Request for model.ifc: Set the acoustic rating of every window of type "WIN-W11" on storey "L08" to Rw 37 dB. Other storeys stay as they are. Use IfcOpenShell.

First a look at what the model holds.

```python
import ifcopenshell
import ifcopenshell.util.element

model = ifcopenshell.open("model.ifc")
print(model.schema)
storey = next(s for s in model.by_type("IfcBuildingStorey") if s.Name == "L08")
windows = [e for e in ifcopenshell.util.element.get_decomposition(storey) if e.is_a("IfcWindow")]
seen = {}
for e in windows:
    element_type = ifcopenshell.util.element.get_type(e)
    key = (element_type.Name if element_type != e and element_type else None, ifcopenshell.util.element.get_pset(e, "Pset_WindowCommon", "AcousticRating"))
    seen[key] = seen.get(key, 0) + 1
for (name, value), count in sorted(seen.items(), key=str):
    print(count, "x", name, "|", value)
```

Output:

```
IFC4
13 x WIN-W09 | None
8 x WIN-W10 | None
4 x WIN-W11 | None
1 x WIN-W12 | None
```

```python
import ifcopenshell
import ifcopenshell.api.pset
import ifcopenshell.util.element

model = ifcopenshell.open("model.ifc")

storey = next(s for s in model.by_type("IfcBuildingStorey") if s.Name == "L08")
windows = [e for e in ifcopenshell.util.element.get_decomposition(storey) if e.is_a("IfcWindow")]

count = 0
for e in windows:
    element_type = ifcopenshell.util.element.get_type(e)
    if element_type in (None, e) or element_type.Name != "WIN-W11":
        continue
    found = ifcopenshell.util.element.get_pset(e, "Pset_WindowCommon", should_inherit=False)
    if found:
        pset = model.by_id(found["id"])
        if len(ifcopenshell.util.element.get_elements_by_pset(pset)) > 1:
            pset = ifcopenshell.api.pset.unshare_pset(model, products=[e], pset=pset)[0]
    else:
        pset = ifcopenshell.api.pset.add_pset(model, product=e, name="Pset_WindowCommon")
    ifcopenshell.api.pset.edit_pset(model, pset=pset, properties={"AcousticRating": "Rw 37 dB"})
    count += 1

print(count, "windows updated")

model.write("model_edited.ifc")
```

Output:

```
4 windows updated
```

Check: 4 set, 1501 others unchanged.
